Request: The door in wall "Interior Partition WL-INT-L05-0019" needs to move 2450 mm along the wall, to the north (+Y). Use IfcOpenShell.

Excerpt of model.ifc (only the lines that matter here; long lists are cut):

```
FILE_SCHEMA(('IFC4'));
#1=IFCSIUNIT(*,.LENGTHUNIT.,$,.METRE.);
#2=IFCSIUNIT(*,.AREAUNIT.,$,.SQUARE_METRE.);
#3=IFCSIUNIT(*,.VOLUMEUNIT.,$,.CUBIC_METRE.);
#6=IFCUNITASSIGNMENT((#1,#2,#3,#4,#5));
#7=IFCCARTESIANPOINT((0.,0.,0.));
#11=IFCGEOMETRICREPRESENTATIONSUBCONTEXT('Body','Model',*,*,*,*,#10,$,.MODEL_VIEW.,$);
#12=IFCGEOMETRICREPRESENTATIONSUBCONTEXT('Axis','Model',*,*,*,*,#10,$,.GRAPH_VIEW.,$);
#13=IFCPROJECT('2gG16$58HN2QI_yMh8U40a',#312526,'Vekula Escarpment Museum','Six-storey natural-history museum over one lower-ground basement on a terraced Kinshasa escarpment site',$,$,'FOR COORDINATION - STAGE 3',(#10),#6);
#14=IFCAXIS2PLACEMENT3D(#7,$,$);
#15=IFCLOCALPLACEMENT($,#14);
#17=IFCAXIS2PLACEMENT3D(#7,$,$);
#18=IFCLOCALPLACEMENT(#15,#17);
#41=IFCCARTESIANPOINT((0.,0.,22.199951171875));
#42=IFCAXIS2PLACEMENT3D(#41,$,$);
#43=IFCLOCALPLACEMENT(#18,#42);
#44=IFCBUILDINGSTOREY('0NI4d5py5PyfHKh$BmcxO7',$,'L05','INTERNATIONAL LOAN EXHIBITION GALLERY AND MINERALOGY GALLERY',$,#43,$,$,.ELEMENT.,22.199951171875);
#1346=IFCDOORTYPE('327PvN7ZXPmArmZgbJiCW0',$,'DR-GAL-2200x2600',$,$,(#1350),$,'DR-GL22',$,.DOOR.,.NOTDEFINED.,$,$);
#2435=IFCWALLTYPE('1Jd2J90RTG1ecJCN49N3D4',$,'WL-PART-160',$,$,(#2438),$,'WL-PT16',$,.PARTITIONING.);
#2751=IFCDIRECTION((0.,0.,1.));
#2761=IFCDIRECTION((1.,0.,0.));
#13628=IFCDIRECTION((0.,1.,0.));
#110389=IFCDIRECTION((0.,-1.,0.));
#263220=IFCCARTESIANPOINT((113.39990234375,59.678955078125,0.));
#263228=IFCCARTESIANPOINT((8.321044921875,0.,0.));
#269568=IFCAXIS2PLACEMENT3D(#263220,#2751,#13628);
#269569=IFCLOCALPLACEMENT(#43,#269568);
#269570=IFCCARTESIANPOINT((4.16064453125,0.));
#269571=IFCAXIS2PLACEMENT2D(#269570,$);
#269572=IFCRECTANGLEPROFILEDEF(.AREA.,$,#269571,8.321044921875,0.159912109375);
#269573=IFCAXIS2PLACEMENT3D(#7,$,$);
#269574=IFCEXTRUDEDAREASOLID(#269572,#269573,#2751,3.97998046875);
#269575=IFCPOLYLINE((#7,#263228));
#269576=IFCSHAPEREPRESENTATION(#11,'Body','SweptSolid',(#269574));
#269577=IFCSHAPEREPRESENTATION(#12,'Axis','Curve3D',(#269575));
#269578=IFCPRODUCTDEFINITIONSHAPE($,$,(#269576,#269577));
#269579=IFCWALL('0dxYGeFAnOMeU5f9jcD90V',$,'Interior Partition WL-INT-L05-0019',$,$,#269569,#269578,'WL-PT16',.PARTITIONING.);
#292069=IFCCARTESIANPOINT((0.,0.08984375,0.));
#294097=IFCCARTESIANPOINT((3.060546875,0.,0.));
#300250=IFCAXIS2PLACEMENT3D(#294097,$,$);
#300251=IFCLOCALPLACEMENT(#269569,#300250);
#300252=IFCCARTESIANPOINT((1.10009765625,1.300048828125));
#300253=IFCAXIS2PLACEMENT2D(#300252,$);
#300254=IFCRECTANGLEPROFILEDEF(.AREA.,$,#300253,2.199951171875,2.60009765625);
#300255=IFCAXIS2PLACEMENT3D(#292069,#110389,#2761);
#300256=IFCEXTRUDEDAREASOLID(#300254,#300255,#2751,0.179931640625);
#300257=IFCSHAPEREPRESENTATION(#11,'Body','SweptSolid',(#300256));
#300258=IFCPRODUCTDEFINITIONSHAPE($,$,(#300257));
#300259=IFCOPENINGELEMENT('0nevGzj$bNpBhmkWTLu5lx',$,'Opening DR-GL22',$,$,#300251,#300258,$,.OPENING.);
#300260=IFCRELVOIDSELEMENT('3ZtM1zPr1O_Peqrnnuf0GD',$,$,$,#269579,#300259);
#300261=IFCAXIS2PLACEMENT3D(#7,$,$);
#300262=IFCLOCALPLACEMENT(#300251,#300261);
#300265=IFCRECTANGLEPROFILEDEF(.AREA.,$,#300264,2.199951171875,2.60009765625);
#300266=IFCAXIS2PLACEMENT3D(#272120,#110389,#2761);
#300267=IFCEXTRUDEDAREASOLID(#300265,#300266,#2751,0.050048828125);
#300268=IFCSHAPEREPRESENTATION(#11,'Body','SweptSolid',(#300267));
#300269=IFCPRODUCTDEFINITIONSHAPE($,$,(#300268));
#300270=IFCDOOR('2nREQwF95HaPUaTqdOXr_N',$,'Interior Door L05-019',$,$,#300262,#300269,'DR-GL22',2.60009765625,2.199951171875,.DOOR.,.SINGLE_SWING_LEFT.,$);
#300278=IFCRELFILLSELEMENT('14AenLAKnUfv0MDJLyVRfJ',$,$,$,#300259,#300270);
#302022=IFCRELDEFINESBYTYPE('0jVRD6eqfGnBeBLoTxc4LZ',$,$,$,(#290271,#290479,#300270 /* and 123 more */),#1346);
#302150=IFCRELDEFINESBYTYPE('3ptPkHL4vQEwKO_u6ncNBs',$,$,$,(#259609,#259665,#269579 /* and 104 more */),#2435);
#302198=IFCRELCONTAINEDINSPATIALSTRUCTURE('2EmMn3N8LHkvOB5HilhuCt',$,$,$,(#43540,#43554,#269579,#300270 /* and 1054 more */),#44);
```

```python
import ifcopenshell
import ifcopenshell.api.geometry
import ifcopenshell.util.placement
import ifcopenshell.util.unit

model = ifcopenshell.open("model.ifc")
unit_scale = ifcopenshell.util.unit.calculate_unit_scale(model)

door = model.by_id(300270)
opening = door.FillsVoids[0].RelatingOpeningElement
wall = opening.VoidsElements[0].RelatingBuildingElement

wall_matrix = ifcopenshell.util.placement.get_local_placement(wall.ObjectPlacement)
shift = wall_matrix[:3, 0] * 2.45 / unit_scale
before = ifcopenshell.util.placement.get_local_placement(door.ObjectPlacement)[:3, 3].copy()

# The door is placed relative to its opening, so it follows when the opening moves.
matrix = ifcopenshell.util.placement.get_local_placement(opening.ObjectPlacement)
matrix[:3, 3] += shift
ifcopenshell.api.geometry.edit_object_placement(
    model, product=opening, matrix=matrix, is_si=False, should_transform_children=True
)

after = ifcopenshell.util.placement.get_local_placement(door.ObjectPlacement)[:3, 3]
print("door moved by", (after - before).round(3) + 0.0)

model.write("model_v2.ifc")
```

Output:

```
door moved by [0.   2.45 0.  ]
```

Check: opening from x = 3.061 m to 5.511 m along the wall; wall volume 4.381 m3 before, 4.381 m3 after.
